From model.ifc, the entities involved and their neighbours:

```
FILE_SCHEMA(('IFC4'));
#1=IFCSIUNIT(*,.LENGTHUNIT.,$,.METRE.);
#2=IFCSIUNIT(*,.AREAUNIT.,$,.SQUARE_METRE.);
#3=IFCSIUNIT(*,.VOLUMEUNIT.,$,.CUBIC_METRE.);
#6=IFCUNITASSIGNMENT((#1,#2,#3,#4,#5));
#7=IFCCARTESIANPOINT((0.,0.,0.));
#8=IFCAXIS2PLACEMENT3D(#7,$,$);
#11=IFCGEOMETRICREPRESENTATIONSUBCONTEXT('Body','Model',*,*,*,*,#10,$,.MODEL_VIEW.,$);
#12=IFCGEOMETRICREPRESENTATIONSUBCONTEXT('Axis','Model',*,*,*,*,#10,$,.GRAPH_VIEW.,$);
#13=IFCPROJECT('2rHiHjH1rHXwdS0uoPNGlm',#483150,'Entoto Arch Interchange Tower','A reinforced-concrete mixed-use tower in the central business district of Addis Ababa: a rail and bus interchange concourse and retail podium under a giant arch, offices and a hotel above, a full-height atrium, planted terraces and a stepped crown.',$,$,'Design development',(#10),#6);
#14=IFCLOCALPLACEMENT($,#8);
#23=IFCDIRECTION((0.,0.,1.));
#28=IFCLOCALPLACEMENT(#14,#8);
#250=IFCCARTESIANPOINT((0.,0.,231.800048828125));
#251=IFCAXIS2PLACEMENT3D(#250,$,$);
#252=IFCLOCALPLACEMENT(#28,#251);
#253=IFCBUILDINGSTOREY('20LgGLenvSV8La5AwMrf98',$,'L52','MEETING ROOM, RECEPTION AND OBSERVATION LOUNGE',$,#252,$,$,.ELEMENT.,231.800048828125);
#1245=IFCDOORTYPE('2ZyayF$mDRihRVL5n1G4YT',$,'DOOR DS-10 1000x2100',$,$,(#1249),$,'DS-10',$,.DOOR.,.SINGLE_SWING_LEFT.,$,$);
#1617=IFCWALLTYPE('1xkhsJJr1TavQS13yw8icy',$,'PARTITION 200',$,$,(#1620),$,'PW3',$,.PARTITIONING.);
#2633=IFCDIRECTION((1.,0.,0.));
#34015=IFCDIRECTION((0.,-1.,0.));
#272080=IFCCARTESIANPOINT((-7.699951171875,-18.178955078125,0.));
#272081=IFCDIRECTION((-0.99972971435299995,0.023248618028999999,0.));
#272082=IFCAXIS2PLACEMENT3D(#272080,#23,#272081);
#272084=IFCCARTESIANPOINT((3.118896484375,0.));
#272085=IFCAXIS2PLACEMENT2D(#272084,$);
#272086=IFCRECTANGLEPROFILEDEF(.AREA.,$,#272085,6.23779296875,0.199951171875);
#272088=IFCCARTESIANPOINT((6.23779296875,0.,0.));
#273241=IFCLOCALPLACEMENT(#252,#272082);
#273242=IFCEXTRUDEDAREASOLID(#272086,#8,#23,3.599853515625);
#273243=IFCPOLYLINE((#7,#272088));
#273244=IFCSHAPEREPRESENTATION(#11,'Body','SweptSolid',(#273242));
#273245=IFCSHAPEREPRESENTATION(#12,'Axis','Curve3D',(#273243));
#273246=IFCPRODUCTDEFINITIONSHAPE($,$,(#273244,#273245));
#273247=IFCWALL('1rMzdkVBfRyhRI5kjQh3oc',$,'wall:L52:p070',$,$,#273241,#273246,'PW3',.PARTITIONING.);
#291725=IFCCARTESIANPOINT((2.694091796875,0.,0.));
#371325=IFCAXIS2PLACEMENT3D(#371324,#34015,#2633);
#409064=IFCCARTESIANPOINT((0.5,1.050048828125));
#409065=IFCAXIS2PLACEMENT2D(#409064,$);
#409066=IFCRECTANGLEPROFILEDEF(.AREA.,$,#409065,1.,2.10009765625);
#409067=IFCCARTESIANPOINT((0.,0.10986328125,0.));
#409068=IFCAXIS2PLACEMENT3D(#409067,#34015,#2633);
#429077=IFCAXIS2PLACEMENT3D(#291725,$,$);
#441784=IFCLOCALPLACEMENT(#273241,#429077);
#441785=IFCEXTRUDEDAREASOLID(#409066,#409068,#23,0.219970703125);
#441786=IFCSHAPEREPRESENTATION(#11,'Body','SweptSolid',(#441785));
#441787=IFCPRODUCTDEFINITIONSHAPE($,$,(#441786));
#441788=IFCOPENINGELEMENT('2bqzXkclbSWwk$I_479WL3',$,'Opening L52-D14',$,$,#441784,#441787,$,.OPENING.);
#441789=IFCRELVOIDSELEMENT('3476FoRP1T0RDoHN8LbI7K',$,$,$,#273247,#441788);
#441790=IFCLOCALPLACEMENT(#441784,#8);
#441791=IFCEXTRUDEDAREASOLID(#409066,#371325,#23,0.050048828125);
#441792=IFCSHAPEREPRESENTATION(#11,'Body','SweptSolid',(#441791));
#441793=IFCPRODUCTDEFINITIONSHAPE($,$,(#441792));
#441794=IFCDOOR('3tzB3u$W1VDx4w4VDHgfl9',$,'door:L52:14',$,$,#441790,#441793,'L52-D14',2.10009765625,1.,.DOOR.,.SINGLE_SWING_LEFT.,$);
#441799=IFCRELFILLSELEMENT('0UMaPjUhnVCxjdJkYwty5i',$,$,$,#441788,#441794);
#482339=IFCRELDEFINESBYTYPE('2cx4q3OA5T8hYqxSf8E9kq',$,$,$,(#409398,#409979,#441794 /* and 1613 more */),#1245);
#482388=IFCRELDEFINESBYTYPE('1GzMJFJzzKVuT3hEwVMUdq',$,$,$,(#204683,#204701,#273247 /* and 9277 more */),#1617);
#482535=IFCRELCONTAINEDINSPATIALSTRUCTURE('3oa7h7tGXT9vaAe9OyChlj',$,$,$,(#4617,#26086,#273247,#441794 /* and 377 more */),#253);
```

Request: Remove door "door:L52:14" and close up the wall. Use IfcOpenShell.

```python
import ifcopenshell
import ifcopenshell.api.feature
import ifcopenshell.api.root
import ifcopenshell.geom
import ifcopenshell.util.shape

model = ifcopenshell.open("model.ifc")
settings = ifcopenshell.geom.settings()


def volume(element):
    """Net volume in cubic metres, openings subtracted."""
    shape = ifcopenshell.geom.create_shape(settings, element)
    return ifcopenshell.util.shape.get_volume(shape.geometry)


door = model.by_guid("3tzB3u$W1VDx4w4VDHgfl9")
opening = door.FillsVoids[0].RelatingOpeningElement
wall = opening.VoidsElements[0].RelatingBuildingElement
before = volume(wall)

ifcopenshell.api.root.remove_product(model, product=door)
ifcopenshell.api.feature.remove_feature(model, feature=opening)

after = volume(wall)

print(f"wall volume {before:.3f} -> {after:.3f} m3")

model.write("model_updated.ifc")
```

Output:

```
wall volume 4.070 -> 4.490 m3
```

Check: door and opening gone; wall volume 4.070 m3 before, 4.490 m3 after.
